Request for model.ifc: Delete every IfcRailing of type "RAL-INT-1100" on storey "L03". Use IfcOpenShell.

First a look at what the model holds.

```python
import ifcopenshell
import ifcopenshell.util.element

model = ifcopenshell.open("model.ifc")
print(model.schema)
storey = next(s for s in model.by_type("IfcBuildingStorey") if s.Name == "L03")
railings = [e for e in ifcopenshell.util.element.get_decomposition(storey) if e.is_a("IfcRailing")]
seen = {}
for e in railings:
    element_type = ifcopenshell.util.element.get_type(e)
    name = element_type.Name if element_type not in (None, e) else None
    seen[name] = seen.get(name, 0) + 1
for name, count in sorted(seen.items(), key=str):
    print(count, "x", name)
```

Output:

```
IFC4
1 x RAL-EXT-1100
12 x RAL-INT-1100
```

```python
import ifcopenshell
import ifcopenshell.api.root
import ifcopenshell.util.element

model = ifcopenshell.open("model.ifc")

storey = next(s for s in model.by_type("IfcBuildingStorey") if s.Name == "L03")
railings = [e for e in ifcopenshell.util.element.get_decomposition(storey) if e.is_a("IfcRailing")]
targets = [e for e in railings if (t := ifcopenshell.util.element.get_type(e)) not in (None, e) and t.Name == "RAL-INT-1100"]

for e in targets:
    ifcopenshell.api.root.remove_product(model, product=e)
print(len(targets), "removed")

model.write("model_edited.ifc")
```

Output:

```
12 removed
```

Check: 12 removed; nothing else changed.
